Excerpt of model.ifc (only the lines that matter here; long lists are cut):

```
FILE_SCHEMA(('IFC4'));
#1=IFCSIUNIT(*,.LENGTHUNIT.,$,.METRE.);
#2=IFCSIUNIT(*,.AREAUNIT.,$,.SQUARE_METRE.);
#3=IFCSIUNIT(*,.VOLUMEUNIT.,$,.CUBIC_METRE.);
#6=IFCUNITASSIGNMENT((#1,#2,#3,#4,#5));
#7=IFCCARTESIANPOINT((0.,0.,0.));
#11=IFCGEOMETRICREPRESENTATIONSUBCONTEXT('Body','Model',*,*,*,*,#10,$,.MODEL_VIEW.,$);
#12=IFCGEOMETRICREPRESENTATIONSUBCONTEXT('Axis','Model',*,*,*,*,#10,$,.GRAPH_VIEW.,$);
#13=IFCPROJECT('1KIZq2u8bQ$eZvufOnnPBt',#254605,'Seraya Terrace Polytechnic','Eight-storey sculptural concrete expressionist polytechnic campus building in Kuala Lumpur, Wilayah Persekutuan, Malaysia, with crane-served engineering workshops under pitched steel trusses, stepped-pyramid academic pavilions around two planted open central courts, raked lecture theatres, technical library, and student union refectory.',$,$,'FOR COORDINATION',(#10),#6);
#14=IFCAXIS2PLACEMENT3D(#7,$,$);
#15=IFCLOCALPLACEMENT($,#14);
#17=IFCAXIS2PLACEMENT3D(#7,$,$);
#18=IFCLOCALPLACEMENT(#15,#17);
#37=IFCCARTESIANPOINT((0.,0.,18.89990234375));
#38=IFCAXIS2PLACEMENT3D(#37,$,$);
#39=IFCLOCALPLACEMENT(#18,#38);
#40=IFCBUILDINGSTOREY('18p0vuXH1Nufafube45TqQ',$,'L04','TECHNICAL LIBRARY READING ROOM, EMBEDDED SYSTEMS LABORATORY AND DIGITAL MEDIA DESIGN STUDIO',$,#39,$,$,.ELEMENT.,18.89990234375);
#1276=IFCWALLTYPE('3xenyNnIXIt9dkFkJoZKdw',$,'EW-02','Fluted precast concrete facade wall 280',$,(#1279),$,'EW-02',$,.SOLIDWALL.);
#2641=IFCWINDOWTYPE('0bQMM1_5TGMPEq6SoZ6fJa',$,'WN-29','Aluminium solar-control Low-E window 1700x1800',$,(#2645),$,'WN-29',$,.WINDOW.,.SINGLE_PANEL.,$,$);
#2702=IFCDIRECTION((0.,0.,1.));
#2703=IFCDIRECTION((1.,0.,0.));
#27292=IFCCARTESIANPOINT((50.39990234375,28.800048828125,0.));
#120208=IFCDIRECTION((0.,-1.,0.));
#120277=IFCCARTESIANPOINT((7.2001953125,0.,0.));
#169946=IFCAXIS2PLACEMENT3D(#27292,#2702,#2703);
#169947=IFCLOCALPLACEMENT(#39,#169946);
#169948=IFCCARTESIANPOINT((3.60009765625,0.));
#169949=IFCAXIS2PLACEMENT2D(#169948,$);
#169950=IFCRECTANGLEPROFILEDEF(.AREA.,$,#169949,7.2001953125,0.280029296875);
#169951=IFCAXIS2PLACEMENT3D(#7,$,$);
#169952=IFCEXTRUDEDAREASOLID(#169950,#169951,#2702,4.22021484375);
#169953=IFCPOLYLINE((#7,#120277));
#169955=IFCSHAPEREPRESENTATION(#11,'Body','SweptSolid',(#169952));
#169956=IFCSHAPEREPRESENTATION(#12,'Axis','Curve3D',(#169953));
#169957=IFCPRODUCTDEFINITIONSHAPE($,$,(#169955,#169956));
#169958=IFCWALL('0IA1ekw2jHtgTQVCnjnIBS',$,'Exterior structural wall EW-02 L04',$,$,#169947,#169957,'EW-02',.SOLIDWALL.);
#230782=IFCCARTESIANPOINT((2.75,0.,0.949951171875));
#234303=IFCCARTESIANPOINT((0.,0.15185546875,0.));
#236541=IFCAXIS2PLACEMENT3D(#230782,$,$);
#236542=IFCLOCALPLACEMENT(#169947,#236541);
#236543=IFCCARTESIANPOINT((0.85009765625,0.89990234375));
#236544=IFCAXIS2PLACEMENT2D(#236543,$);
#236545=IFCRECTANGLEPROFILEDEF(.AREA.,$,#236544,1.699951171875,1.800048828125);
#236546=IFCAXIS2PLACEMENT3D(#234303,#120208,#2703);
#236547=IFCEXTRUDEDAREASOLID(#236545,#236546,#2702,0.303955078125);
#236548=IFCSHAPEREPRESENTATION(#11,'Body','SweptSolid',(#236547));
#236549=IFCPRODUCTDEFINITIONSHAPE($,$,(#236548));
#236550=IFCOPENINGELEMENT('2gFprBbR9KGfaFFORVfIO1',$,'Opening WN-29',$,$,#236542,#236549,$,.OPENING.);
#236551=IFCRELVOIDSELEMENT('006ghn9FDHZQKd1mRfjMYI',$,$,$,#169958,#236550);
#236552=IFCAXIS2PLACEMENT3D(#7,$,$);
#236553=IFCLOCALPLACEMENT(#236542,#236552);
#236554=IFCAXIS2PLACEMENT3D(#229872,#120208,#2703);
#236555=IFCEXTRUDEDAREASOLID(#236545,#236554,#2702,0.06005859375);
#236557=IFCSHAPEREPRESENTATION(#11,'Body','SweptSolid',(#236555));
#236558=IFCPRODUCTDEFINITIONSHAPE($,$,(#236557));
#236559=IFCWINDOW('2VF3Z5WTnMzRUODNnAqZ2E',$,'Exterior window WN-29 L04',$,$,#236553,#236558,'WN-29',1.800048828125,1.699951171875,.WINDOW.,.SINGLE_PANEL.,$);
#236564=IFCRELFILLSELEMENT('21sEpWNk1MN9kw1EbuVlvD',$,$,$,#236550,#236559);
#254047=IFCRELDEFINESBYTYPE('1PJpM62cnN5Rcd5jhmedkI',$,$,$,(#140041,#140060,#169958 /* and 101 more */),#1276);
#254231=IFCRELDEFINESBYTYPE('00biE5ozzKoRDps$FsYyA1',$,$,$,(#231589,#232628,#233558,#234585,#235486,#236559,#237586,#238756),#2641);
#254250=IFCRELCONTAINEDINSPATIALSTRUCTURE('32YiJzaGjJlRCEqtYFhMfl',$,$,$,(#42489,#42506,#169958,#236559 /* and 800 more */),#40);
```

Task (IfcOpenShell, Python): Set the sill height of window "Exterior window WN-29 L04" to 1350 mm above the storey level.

```python
import numpy as np
import ifcopenshell
import ifcopenshell.api.geometry
import ifcopenshell.geom
import ifcopenshell.util.element
import ifcopenshell.util.placement
import ifcopenshell.util.shape
import ifcopenshell.util.unit

model = ifcopenshell.open("model.ifc")
unit_scale = ifcopenshell.util.unit.calculate_unit_scale(model)

window = model.by_guid("2VF3Z5WTnMzRUODNnAqZ2E")
opening = window.FillsVoids[0].RelatingOpeningElement
storey = ifcopenshell.util.element.get_container(window, ifc_class="IfcBuildingStorey")
level = ifcopenshell.util.placement.get_local_placement(storey.ObjectPlacement)[2, 3]

# The opening's origin need not be at the sill, so measure its lowest point.
shape = ifcopenshell.geom.create_shape(ifcopenshell.geom.settings(), opening)
bottom = ifcopenshell.util.shape.get_shape_bottom_elevation(shape, shape.geometry) / unit_scale
dz = level + 1.35 - bottom

shift = np.array([0.0, 0.0, dz])
# The window is placed relative to its opening, so it follows when the opening moves.
matrix = ifcopenshell.util.placement.get_local_placement(opening.ObjectPlacement)
matrix[:3, 3] += shift
ifcopenshell.api.geometry.edit_object_placement(
    model, product=opening, matrix=matrix, is_si=False, should_transform_children=True
)

print(f"moved by {dz * unit_scale:+.3f} m")

model.write("model-out.ifc")
```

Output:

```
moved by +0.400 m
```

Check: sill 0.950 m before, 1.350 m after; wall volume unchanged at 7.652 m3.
